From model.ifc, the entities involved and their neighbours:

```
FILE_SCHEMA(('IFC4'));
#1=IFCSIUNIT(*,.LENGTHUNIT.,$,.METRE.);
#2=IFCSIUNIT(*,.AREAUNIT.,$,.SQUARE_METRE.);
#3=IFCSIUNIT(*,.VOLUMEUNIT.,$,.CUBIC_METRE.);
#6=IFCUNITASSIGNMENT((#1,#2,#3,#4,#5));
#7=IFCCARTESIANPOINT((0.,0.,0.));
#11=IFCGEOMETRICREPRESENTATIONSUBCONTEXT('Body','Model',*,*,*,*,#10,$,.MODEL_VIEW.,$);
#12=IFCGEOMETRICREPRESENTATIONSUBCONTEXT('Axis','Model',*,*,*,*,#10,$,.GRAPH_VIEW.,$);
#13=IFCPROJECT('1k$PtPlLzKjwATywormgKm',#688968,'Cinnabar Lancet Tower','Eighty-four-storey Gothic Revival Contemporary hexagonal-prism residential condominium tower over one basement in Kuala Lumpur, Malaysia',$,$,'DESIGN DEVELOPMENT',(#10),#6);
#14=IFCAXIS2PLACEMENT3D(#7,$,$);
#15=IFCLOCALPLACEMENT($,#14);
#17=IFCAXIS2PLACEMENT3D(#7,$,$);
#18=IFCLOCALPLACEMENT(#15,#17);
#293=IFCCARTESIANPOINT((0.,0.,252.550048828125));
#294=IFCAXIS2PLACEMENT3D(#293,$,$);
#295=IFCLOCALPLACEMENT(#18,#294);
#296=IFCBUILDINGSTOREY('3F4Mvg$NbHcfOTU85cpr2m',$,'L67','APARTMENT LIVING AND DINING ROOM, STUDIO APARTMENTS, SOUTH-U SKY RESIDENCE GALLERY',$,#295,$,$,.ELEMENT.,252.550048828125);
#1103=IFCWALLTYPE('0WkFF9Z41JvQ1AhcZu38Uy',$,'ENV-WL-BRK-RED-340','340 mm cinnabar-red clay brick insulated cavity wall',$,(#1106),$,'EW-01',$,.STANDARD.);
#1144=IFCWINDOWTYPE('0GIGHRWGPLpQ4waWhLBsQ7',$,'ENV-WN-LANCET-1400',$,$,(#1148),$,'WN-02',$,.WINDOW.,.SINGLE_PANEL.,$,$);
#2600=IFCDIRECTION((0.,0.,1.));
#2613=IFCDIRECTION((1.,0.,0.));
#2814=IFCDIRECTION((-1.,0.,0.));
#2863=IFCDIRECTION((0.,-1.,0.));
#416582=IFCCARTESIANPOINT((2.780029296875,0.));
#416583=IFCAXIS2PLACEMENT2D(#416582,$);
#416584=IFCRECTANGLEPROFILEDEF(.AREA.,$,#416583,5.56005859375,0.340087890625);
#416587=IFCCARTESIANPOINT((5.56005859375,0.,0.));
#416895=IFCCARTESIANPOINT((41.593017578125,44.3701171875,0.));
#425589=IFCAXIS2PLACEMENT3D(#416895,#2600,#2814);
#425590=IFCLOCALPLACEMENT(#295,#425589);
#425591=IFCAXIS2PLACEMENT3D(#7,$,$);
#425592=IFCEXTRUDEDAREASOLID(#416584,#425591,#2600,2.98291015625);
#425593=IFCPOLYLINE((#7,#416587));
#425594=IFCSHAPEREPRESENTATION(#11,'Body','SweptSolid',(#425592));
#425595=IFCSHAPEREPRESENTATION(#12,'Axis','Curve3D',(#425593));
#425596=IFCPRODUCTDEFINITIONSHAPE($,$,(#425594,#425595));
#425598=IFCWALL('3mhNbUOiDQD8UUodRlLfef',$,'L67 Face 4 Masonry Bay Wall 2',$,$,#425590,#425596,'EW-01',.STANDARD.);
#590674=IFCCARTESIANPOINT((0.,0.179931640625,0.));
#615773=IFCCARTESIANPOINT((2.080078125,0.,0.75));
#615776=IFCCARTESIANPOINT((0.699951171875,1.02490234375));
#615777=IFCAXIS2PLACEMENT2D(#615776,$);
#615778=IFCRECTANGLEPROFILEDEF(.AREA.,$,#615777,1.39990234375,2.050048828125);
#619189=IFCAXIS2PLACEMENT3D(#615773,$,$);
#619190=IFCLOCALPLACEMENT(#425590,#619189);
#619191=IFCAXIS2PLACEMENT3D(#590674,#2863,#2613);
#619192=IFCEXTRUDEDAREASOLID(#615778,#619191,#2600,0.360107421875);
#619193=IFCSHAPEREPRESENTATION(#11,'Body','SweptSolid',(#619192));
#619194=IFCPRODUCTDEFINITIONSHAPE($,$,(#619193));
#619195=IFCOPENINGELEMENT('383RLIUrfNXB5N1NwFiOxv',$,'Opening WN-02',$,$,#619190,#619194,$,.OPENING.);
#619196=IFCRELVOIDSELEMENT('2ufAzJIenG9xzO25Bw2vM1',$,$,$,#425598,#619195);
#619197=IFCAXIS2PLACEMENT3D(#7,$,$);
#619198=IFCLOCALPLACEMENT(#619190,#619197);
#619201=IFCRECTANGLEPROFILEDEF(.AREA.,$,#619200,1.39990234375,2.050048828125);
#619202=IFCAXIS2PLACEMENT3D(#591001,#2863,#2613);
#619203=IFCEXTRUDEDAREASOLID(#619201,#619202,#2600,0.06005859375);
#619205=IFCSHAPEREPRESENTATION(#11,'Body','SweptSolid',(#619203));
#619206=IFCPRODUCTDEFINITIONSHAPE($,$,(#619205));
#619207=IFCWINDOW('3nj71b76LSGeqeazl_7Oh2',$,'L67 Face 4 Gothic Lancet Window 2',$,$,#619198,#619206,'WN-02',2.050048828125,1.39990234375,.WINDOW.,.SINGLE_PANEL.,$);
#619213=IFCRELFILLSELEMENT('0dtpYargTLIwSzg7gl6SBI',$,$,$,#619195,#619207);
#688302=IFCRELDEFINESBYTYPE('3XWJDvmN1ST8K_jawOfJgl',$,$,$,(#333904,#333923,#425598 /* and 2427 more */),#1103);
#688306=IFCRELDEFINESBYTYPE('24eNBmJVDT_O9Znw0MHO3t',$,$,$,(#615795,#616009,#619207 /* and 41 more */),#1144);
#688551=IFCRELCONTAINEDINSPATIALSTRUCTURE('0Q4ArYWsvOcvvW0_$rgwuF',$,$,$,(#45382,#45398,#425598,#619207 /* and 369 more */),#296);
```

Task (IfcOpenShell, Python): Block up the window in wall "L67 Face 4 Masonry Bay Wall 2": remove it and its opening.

```python
import ifcopenshell
import ifcopenshell.api.feature
import ifcopenshell.api.root
import ifcopenshell.geom
import ifcopenshell.util.shape

model = ifcopenshell.open("model.ifc")
settings = ifcopenshell.geom.settings()


def volume(element):
    """Net volume in cubic metres, openings subtracted."""
    shape = ifcopenshell.geom.create_shape(settings, element)
    return ifcopenshell.util.shape.get_volume(shape.geometry)


window = model.by_guid("3nj71b76LSGeqeazl_7Oh2")
opening = window.FillsVoids[0].RelatingOpeningElement
wall = opening.VoidsElements[0].RelatingBuildingElement
before = volume(wall)

ifcopenshell.api.root.remove_product(model, product=window)
ifcopenshell.api.feature.remove_feature(model, feature=opening)

after = volume(wall)

print(f"wall volume {before:.3f} -> {after:.3f} m3")

model.write("model-out.ifc")
```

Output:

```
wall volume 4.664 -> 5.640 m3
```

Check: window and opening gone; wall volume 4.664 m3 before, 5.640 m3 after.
